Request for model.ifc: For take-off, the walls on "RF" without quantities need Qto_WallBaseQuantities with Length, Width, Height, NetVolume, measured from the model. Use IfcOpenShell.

First a look at what the model holds.

```python
import ifcopenshell
import ifcopenshell.util.element
import ifcopenshell.util.unit

model = ifcopenshell.open("model.ifc")
print(model.schema)
for unit_type in ("LENGTHUNIT", "AREAUNIT", "VOLUMEUNIT"):
    print(unit_type, ifcopenshell.util.unit.calculate_unit_scale(model, unit_type))
storey = next(s for s in model.by_type("IfcBuildingStorey") if s.Name == "RF")
walls = [e for e in ifcopenshell.util.element.get_decomposition(storey) if e.is_a("IfcWall")]
for e in sorted(walls, key=lambda e: e.id()):
    print(e.id(), e.is_a(), e.Name, list(ifcopenshell.util.element.get_psets(e, qtos_only=True)), sep=" | ")
```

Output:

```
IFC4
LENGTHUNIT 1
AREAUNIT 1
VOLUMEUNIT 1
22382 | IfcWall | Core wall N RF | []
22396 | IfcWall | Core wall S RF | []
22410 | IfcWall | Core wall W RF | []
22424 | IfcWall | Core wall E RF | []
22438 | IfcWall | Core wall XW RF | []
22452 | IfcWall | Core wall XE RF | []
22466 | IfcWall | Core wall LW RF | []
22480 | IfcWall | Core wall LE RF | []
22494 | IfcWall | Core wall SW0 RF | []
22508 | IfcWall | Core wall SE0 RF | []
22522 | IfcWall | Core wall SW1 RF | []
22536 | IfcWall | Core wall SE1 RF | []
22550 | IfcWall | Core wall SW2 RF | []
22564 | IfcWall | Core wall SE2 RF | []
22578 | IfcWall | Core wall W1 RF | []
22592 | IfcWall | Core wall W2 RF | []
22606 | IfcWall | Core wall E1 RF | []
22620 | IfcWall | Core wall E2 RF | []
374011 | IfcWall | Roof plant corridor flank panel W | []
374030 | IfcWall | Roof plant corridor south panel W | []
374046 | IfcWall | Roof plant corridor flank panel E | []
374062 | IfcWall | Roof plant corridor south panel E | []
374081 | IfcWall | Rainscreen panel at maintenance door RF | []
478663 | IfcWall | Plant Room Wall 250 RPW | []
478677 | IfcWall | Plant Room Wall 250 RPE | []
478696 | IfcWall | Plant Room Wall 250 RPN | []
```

```python
import ifcopenshell
import ifcopenshell.api.pset
import ifcopenshell.geom
import ifcopenshell.util.element
import ifcopenshell.util.shape
import ifcopenshell.util.unit

model = ifcopenshell.open("model.ifc")
unit_scale = ifcopenshell.util.unit.calculate_unit_scale(model)
volume_scale = ifcopenshell.util.unit.calculate_unit_scale(model, "VOLUMEUNIT")
settings = ifcopenshell.geom.settings()

storey = next(s for s in model.by_type("IfcBuildingStorey") if s.Name == "RF")
walls = [e for e in ifcopenshell.util.element.get_decomposition(storey) if e.is_a("IfcWall")]

for e in sorted(walls, key=lambda e: e.id()):
    if ifcopenshell.util.element.get_psets(e, qtos_only=True, should_inherit=False):
        continue
    # Geometry comes back in metres, in the element's own axes.
    shape = ifcopenshell.geom.create_shape(settings, e)
    values = {
        "Length": ifcopenshell.util.shape.get_x(shape.geometry) / unit_scale,
        "Width": ifcopenshell.util.shape.get_y(shape.geometry) / unit_scale,
        "Height": ifcopenshell.util.shape.get_z(shape.geometry) / unit_scale,
        "NetVolume": ifcopenshell.util.shape.get_volume(shape.geometry) / volume_scale,
    }
    qto = ifcopenshell.api.pset.add_qto(model, product=e, name="Qto_WallBaseQuantities")
    ifcopenshell.api.pset.edit_qto(model, qto=qto, properties=values)
    print(e.id(), {k: round(v, 3) for k, v in values.items()})

model.write("model_updated.ifc")
```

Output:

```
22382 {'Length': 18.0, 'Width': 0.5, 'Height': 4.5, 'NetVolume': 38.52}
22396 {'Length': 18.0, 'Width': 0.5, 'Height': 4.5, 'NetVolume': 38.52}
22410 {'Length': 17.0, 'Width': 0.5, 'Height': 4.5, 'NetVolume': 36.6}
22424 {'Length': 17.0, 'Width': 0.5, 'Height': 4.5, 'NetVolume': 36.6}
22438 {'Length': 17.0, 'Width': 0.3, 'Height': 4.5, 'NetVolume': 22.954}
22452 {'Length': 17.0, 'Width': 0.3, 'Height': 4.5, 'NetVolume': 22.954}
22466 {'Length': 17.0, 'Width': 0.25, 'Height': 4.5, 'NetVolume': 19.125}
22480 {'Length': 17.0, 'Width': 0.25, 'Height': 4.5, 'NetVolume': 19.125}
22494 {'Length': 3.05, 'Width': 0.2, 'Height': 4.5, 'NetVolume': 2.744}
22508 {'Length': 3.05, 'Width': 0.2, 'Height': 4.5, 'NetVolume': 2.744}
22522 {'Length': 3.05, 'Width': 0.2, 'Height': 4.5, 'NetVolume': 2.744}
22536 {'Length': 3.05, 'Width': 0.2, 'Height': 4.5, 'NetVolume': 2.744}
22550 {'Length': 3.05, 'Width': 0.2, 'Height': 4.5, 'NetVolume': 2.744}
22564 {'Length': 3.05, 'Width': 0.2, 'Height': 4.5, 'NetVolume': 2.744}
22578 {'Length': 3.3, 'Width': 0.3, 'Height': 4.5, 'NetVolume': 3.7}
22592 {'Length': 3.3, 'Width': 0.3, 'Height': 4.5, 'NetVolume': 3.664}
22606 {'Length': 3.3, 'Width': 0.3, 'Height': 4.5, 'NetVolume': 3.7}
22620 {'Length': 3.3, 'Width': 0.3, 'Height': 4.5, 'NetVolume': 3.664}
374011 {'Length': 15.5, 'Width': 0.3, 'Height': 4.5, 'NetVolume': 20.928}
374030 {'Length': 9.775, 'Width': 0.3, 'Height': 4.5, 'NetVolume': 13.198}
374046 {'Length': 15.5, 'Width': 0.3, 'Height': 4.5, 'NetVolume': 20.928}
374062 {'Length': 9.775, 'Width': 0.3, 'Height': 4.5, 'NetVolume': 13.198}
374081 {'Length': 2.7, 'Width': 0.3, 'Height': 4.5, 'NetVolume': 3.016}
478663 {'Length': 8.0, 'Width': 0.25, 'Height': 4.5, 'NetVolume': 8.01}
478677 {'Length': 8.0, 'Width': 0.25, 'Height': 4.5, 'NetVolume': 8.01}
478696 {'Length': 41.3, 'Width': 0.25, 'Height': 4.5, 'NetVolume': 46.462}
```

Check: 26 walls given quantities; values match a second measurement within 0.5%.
